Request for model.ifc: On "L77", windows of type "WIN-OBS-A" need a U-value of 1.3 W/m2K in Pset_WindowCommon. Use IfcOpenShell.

First a look at what the model holds.

```python
import ifcopenshell
import ifcopenshell.util.element

model = ifcopenshell.open("model.ifc")
print(model.schema)
storey = next(s for s in model.by_type("IfcBuildingStorey") if s.Name == "L77")
windows = [e for e in ifcopenshell.util.element.get_decomposition(storey) if e.is_a("IfcWindow")]
seen = {}
for e in windows:
    element_type = ifcopenshell.util.element.get_type(e)
    key = (element_type.Name if element_type != e and element_type else None, ifcopenshell.util.element.get_pset(e, "Pset_WindowCommon", "ThermalTransmittance"))
    seen[key] = seen.get(key, 0) + 1
for (name, value), count in sorted(seen.items(), key=str):
    print(count, "x", name, "|", value)
```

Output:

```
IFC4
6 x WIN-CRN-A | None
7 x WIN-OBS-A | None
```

```python
import ifcopenshell
import ifcopenshell.api.pset
import ifcopenshell.util.element

model = ifcopenshell.open("model.ifc")

storey = next(s for s in model.by_type("IfcBuildingStorey") if s.Name == "L77")
windows = [e for e in ifcopenshell.util.element.get_decomposition(storey) if e.is_a("IfcWindow")]

count = 0
for e in windows:
    element_type = ifcopenshell.util.element.get_type(e)
    if element_type in (None, e) or element_type.Name != "WIN-OBS-A":
        continue
    # add_pset returns the element's existing set when there is one.
    pset = ifcopenshell.api.pset.add_pset(model, product=e, name="Pset_WindowCommon")
    ifcopenshell.api.pset.edit_pset(model, pset=pset, properties={"ThermalTransmittance": 1.3})
    count += 1

print(count, "windows updated")

model.write("model_updated.ifc")
```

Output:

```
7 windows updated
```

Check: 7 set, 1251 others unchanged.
